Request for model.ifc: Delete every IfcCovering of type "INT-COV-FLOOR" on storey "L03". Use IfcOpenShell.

First a look at what the model holds.

```python
import ifcopenshell
import ifcopenshell.util.element

model = ifcopenshell.open("model.ifc")
print(model.schema)
storey = next(s for s in model.by_type("IfcBuildingStorey") if s.Name == "L03")
coverings = [e for e in ifcopenshell.util.element.get_decomposition(storey) if e.is_a("IfcCovering")]
seen = {}
for e in coverings:
    element_type = ifcopenshell.util.element.get_type(e)
    name = element_type.Name if element_type not in (None, e) else None
    seen[name] = seen.get(name, 0) + 1
for name, count in sorted(seen.items(), key=str):
    print(count, "x", name)
```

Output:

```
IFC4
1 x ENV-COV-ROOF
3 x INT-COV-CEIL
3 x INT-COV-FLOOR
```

```python
import ifcopenshell
import ifcopenshell.api.root
import ifcopenshell.util.element

model = ifcopenshell.open("model.ifc")

storey = next(s for s in model.by_type("IfcBuildingStorey") if s.Name == "L03")
coverings = [e for e in ifcopenshell.util.element.get_decomposition(storey) if e.is_a("IfcCovering")]
targets = [e for e in coverings if (t := ifcopenshell.util.element.get_type(e)) not in (None, e) and t.Name == "INT-COV-FLOOR"]

for e in targets:
    ifcopenshell.api.root.remove_product(model, product=e)
print(len(targets), "removed")

model.write("model_updated.ifc")
```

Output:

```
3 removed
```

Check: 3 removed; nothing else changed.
